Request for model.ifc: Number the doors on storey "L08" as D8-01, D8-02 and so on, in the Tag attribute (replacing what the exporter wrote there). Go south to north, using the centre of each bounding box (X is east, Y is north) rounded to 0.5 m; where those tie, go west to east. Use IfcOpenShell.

First a look at what the model holds.

```python
import ifcopenshell
import ifcopenshell.util.element
import ifcopenshell.util.placement

model = ifcopenshell.open("model.ifc")
print(model.schema)
storey = next(s for s in model.by_type("IfcBuildingStorey") if s.Name == "L08")
doors = [e for e in ifcopenshell.util.element.get_decomposition(storey) if e.is_a("IfcDoor")]
for e in sorted(doors, key=lambda e: e.id()):
    origin = ifcopenshell.util.placement.get_local_placement(e.ObjectPlacement)[:3, 3]
    print(e.id(), e.Tag, e.Name, origin.round(2) + 0.0, sep=" | ")
```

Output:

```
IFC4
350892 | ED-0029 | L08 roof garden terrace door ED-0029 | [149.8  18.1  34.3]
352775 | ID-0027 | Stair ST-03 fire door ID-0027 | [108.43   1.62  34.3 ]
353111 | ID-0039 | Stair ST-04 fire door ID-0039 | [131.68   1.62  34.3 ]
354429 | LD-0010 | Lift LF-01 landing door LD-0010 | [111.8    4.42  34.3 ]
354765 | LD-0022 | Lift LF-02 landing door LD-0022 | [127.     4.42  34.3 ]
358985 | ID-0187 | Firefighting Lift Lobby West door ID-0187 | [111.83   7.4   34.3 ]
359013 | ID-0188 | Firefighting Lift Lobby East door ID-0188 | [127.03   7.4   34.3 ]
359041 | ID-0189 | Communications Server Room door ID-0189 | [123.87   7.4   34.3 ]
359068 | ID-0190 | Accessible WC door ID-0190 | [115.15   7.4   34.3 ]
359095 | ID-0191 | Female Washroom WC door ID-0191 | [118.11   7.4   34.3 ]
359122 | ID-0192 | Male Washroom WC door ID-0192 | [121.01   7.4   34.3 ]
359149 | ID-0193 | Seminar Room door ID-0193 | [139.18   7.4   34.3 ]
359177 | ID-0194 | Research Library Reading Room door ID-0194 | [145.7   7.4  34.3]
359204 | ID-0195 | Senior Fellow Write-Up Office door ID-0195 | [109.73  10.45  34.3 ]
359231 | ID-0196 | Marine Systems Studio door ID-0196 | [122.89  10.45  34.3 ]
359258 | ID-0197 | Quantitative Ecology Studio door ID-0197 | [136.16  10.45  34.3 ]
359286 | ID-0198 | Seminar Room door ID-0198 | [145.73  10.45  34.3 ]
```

```python
import ifcopenshell
import ifcopenshell.geom
import ifcopenshell.util.element
import ifcopenshell.util.shape

model = ifcopenshell.open("model.ifc")
settings = ifcopenshell.geom.settings()
settings.set("use-world-coords", True)


def centre(element):
    shape = ifcopenshell.geom.create_shape(settings, element)
    return ifcopenshell.util.shape.get_bbox_centroid(shape.geometry)


storey = next(s for s in model.by_type("IfcBuildingStorey") if s.Name == "L08")
doors = [e for e in ifcopenshell.util.element.get_decomposition(storey) if e.is_a("IfcDoor")]

# Insertion points can sit at a corner or the storey origin, so sort by the geometry (in metres).
centres = {e: centre(e) for e in doors}
doors.sort(key=lambda e: (round(centres[e][1] / 0.5), centres[e][0]))

for i, e in enumerate(doors, start=1):
    number = f"D8-{i:02d}"
    e.Tag = number
    print(e.id(), number)

model.write("model-out.ifc")
```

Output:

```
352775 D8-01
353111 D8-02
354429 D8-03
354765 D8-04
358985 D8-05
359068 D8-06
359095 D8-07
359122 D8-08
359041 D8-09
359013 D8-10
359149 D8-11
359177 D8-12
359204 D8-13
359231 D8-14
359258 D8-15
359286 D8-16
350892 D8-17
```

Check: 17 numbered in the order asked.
